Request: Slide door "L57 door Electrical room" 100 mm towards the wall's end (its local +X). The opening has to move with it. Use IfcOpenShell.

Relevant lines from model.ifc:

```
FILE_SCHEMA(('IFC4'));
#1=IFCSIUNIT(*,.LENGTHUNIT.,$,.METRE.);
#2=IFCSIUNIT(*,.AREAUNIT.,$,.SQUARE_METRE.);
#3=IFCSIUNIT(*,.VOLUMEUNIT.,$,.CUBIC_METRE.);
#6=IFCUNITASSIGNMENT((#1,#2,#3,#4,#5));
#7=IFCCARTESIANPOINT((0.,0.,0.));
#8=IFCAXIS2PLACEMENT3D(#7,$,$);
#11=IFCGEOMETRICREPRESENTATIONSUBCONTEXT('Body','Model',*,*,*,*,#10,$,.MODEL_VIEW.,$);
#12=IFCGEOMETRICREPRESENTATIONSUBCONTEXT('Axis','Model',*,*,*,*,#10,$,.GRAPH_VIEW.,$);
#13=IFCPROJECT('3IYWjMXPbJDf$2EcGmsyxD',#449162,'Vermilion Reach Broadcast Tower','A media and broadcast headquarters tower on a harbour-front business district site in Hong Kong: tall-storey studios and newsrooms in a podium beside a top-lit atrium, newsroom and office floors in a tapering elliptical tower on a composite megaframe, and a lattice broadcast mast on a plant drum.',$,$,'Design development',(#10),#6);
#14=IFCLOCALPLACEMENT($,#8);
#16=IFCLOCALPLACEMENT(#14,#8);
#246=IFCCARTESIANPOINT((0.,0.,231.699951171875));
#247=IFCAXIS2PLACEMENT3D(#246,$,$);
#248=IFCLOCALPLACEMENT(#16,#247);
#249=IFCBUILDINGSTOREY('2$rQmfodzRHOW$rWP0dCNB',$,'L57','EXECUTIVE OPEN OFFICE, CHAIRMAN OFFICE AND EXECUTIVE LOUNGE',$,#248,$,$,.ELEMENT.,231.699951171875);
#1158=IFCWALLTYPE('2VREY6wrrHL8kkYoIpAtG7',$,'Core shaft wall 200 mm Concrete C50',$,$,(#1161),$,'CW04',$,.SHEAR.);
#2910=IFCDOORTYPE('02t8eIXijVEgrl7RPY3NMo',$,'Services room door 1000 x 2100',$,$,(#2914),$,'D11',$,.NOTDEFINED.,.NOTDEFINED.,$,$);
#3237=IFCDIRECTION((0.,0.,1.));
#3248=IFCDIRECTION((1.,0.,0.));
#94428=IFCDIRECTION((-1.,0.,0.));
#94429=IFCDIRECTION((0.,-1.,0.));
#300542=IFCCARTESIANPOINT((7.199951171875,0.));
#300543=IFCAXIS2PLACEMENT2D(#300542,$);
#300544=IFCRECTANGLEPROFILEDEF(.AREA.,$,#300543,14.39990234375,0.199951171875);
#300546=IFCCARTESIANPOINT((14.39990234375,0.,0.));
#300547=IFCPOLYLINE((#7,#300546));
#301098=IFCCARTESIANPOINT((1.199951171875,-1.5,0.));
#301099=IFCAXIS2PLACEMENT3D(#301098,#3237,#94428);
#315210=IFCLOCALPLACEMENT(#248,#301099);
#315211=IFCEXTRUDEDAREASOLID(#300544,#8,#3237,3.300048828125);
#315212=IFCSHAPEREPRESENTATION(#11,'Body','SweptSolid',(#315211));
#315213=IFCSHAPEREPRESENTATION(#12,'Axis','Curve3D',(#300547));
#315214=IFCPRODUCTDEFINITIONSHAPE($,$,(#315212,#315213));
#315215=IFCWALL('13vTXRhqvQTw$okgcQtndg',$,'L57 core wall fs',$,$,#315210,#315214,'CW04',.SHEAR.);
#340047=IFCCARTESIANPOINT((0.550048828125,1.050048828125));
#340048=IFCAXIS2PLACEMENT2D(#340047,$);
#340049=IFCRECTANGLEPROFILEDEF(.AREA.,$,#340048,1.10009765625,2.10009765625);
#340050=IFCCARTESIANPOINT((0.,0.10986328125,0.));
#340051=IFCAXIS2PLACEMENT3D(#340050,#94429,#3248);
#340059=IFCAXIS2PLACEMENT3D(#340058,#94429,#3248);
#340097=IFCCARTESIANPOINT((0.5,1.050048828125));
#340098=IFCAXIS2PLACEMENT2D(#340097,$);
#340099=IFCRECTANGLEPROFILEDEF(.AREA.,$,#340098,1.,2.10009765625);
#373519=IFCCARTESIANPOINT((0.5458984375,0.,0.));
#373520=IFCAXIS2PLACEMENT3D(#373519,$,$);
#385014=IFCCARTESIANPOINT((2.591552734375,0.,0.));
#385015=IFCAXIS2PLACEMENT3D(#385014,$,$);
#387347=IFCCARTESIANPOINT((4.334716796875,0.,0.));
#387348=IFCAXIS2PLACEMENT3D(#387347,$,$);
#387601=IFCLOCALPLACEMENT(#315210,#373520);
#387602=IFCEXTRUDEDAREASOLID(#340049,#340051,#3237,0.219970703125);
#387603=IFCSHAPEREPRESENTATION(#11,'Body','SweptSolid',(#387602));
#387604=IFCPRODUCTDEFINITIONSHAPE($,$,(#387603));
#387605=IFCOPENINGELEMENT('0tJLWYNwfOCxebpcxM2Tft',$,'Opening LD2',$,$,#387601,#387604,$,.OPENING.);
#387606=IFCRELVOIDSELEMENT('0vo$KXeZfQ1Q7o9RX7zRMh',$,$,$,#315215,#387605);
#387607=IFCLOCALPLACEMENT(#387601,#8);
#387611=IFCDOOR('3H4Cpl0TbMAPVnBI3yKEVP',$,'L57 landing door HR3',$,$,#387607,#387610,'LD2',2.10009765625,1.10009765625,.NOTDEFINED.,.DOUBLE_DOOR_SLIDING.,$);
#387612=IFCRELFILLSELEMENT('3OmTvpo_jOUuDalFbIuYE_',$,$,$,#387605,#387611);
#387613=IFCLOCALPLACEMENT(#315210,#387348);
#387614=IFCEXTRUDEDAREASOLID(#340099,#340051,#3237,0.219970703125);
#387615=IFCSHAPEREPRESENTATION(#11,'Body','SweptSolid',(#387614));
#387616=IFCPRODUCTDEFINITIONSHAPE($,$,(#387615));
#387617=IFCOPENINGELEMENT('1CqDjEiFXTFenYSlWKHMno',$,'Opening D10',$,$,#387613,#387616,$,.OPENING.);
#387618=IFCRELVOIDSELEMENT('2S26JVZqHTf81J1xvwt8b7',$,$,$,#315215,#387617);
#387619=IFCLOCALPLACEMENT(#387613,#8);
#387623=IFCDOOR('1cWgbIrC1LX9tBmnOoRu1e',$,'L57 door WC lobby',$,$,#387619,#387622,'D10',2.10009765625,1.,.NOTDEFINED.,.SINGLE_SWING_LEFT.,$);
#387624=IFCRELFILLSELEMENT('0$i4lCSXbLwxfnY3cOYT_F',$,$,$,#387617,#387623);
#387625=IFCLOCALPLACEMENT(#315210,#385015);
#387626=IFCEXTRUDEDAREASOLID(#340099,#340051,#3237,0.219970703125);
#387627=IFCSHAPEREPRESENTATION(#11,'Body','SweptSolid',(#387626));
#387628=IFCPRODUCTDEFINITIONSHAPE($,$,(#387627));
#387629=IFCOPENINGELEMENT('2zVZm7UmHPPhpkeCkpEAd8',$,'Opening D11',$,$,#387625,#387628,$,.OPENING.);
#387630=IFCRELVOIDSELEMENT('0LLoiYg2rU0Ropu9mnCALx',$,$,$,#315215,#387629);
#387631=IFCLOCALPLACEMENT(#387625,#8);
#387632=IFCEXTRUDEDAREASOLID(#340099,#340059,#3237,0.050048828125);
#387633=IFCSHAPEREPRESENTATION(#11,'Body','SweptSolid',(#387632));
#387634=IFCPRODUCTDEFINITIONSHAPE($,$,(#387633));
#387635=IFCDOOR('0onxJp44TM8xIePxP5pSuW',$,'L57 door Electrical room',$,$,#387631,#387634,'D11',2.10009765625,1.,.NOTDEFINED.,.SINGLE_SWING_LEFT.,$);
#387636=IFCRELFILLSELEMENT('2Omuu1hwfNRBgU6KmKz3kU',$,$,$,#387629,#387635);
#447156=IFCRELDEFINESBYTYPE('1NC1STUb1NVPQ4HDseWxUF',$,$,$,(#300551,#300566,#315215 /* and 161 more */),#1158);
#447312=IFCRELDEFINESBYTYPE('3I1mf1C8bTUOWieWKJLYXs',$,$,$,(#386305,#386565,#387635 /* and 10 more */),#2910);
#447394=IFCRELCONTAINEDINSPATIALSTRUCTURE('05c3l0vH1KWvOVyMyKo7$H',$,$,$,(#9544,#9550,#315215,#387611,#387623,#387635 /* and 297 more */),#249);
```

```python
import ifcopenshell
import ifcopenshell.api.geometry
import ifcopenshell.util.placement
import ifcopenshell.util.unit

model = ifcopenshell.open("model.ifc")
unit_scale = ifcopenshell.util.unit.calculate_unit_scale(model)

door = model.by_guid("0onxJp44TM8xIePxP5pSuW")
opening = door.FillsVoids[0].RelatingOpeningElement
wall = opening.VoidsElements[0].RelatingBuildingElement

wall_matrix = ifcopenshell.util.placement.get_local_placement(wall.ObjectPlacement)
shift = wall_matrix[:3, 0] * 0.1 / unit_scale
before = ifcopenshell.util.placement.get_local_placement(door.ObjectPlacement)[:3, 3].copy()

# The door is placed relative to its opening, so it follows when the opening moves.
matrix = ifcopenshell.util.placement.get_local_placement(opening.ObjectPlacement)
matrix[:3, 3] += shift
ifcopenshell.api.geometry.edit_object_placement(
    model, product=opening, matrix=matrix, is_si=False, should_transform_children=True
)

after = ifcopenshell.util.placement.get_local_placement(door.ObjectPlacement)[:3, 3]
print("door moved by", (after - before).round(3) + 0.0)

model.write("model_rev.ifc")
```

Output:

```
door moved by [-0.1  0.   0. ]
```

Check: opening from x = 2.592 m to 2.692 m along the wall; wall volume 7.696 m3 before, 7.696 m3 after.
